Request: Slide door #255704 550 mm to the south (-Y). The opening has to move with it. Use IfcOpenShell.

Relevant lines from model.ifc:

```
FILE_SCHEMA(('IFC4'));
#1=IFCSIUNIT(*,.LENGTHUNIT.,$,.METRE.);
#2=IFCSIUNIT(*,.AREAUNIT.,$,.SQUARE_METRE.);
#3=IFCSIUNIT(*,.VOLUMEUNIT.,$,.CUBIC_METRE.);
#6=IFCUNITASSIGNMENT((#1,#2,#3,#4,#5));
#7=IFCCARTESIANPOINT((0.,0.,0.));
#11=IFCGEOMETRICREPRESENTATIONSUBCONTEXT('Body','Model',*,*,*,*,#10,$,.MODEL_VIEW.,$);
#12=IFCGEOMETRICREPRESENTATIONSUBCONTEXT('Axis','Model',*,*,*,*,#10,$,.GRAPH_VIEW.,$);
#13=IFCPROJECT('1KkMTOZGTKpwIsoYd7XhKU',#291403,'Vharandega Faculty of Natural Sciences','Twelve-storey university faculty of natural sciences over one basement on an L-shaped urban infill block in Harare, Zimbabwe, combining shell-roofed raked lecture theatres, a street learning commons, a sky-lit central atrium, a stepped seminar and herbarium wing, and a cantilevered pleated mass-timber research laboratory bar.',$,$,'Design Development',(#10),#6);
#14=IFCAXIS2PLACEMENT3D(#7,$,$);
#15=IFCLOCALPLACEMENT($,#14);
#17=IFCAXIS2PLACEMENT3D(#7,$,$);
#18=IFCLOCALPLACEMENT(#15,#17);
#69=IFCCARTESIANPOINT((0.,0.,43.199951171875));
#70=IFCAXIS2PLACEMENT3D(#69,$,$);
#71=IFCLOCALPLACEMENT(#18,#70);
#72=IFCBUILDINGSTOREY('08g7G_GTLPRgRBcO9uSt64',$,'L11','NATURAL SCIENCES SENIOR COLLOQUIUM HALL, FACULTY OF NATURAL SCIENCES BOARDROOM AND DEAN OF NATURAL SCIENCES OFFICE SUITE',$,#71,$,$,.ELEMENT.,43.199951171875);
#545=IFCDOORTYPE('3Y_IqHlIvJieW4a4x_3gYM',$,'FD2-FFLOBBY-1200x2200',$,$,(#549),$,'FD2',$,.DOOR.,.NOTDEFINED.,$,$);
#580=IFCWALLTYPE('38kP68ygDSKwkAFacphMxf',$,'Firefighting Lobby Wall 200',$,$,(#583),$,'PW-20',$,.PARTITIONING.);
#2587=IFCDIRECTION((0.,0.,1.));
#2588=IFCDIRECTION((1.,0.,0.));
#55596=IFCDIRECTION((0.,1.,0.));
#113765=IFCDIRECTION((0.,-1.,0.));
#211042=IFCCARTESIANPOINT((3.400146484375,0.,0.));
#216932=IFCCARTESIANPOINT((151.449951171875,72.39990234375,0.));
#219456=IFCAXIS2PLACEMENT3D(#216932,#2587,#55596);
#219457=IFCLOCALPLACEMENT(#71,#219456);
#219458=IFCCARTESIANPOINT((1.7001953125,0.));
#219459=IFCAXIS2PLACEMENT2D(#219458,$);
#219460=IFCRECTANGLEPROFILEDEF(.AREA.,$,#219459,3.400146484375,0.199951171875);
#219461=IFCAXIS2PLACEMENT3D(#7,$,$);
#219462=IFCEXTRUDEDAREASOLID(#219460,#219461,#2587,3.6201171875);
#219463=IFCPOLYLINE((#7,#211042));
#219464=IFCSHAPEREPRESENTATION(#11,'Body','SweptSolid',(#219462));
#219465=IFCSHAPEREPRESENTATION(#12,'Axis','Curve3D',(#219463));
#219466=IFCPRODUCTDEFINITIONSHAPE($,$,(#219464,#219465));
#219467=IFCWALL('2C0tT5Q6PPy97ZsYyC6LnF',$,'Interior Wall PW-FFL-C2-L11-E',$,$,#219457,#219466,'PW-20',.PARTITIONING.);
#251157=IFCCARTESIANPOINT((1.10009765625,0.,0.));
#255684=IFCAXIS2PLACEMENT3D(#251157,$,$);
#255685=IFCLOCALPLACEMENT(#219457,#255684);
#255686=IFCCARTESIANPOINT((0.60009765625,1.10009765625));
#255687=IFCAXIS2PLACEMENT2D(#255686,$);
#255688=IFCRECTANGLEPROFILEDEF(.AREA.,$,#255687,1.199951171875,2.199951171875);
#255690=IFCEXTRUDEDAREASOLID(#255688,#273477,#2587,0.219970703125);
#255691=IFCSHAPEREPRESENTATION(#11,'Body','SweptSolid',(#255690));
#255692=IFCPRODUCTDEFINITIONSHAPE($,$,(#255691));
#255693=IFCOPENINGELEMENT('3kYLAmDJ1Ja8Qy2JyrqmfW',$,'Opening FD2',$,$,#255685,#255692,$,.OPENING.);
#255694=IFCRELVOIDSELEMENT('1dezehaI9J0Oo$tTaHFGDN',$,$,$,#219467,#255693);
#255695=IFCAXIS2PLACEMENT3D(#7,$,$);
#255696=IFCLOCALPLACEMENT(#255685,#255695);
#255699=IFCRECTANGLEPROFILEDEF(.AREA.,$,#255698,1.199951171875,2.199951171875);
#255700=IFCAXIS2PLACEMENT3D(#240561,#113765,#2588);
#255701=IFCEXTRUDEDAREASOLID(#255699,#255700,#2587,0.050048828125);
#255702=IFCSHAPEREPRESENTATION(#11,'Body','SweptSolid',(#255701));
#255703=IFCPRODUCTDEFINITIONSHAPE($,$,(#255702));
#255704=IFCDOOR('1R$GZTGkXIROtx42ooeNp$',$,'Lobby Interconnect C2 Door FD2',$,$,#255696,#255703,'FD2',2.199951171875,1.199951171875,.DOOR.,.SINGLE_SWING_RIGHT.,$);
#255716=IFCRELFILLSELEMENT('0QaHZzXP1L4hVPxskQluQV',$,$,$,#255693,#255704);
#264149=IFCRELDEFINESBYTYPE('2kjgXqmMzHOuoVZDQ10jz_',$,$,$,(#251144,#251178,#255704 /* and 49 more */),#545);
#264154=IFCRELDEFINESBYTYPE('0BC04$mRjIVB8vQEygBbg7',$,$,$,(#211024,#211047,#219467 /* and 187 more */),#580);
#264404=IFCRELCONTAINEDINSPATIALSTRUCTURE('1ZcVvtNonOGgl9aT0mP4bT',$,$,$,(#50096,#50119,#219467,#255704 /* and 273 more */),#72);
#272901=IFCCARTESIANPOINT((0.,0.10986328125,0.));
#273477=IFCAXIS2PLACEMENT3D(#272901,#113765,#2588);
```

```python
import ifcopenshell
import ifcopenshell.api.geometry
import ifcopenshell.util.placement

model = ifcopenshell.open("model.ifc")

door = model.by_id(255704)
opening = door.FillsVoids[0].RelatingOpeningElement
wall = opening.VoidsElements[0].RelatingBuildingElement

wall_matrix = ifcopenshell.util.placement.get_local_placement(wall.ObjectPlacement)
shift = wall_matrix[:3, 0] * -0.55
before = ifcopenshell.util.placement.get_local_placement(door.ObjectPlacement)[:3, 3].copy()

# The door is placed relative to its opening, so it follows when the opening moves.
matrix = ifcopenshell.util.placement.get_local_placement(opening.ObjectPlacement)
matrix[:3, 3] += shift
ifcopenshell.api.geometry.edit_object_placement(
    model, product=opening, matrix=matrix, is_si=False, should_transform_children=True
)

after = ifcopenshell.util.placement.get_local_placement(door.ObjectPlacement)[:3, 3]
print("door moved by", (after - before).round(3) + 0.0)

model.write("model_edited.ifc")
```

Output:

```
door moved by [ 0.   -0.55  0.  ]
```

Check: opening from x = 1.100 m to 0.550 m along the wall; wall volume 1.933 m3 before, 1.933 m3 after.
